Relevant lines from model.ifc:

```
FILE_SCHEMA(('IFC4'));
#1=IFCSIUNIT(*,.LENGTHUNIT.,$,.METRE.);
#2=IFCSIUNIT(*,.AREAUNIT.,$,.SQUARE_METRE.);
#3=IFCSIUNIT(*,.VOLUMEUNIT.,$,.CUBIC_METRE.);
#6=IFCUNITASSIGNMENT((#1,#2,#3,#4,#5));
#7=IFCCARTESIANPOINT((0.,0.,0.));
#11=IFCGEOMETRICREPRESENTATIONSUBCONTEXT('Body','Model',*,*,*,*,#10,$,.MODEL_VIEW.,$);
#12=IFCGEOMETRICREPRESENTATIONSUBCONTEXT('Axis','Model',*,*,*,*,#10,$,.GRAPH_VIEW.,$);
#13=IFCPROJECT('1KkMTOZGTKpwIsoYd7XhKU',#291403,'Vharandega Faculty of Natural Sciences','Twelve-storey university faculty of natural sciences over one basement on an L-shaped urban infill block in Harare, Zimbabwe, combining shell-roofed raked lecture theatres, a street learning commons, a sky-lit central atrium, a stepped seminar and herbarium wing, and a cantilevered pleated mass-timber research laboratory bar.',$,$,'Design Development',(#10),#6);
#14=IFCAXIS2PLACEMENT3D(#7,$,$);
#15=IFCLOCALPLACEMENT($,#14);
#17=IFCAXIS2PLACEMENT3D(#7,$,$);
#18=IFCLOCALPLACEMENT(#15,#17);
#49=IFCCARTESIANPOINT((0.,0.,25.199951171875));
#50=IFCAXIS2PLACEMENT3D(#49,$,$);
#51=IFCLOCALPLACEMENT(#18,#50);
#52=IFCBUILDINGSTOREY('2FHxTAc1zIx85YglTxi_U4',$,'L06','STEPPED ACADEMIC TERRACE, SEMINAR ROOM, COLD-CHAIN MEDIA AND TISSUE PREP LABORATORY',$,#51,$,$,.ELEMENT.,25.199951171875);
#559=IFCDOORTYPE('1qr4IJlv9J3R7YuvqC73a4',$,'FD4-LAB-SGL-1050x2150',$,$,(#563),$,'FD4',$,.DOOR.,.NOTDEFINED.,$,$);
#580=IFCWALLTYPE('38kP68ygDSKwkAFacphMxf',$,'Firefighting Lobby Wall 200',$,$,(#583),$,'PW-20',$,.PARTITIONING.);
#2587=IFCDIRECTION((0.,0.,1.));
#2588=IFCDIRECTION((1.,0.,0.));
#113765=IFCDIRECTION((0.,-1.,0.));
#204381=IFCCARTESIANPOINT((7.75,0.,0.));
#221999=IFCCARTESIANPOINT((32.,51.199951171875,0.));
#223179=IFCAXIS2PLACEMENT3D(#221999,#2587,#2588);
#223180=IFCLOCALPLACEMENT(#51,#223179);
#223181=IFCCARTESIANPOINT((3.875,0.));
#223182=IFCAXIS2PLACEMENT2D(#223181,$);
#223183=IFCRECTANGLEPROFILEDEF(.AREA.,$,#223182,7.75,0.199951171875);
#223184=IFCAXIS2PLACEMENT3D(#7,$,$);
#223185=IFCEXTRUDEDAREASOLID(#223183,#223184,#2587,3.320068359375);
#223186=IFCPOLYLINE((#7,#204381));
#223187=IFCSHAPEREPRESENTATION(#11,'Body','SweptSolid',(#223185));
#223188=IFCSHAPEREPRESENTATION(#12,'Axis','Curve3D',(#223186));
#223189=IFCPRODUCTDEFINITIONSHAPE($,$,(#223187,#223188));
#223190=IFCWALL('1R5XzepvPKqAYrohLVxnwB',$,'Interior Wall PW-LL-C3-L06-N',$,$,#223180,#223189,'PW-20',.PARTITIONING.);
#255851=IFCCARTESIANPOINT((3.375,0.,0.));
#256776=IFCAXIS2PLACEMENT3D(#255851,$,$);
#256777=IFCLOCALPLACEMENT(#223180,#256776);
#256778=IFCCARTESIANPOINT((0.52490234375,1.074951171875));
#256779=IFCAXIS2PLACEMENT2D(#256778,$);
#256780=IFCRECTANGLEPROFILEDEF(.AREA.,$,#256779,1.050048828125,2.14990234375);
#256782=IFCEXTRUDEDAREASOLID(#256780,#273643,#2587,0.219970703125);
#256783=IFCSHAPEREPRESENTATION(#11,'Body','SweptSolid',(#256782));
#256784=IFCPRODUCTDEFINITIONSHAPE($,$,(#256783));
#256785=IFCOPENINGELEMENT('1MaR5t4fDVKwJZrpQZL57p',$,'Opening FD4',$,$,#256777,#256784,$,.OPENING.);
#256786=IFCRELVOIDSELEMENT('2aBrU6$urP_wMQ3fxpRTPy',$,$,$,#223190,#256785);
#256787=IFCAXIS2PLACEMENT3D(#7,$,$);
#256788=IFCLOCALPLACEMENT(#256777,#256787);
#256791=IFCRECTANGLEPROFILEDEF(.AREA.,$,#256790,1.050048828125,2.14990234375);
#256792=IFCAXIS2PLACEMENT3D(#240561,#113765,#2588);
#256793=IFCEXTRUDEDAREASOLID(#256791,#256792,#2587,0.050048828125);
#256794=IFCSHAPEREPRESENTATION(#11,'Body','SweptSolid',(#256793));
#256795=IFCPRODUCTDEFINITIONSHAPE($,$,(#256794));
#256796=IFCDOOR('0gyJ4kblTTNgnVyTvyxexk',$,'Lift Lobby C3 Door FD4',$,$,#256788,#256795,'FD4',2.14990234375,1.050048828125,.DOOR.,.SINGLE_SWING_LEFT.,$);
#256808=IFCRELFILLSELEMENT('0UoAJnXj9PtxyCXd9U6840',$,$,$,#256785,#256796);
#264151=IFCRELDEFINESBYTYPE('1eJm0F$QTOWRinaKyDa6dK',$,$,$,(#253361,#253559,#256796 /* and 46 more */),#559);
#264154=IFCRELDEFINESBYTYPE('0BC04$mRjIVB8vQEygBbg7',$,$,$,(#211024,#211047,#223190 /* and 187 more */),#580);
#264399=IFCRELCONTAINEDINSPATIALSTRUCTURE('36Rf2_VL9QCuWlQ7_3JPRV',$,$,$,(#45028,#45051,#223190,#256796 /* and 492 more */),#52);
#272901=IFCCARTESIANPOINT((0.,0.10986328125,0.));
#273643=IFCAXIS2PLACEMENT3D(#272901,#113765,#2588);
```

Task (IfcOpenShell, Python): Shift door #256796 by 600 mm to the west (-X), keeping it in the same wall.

```python
import ifcopenshell
import ifcopenshell.api.geometry
import ifcopenshell.util.placement

model = ifcopenshell.open("model.ifc")

door = model.by_guid("0gyJ4kblTTNgnVyTvyxexk")
opening = door.FillsVoids[0].RelatingOpeningElement
wall = opening.VoidsElements[0].RelatingBuildingElement

wall_matrix = ifcopenshell.util.placement.get_local_placement(wall.ObjectPlacement)
shift = wall_matrix[:3, 0] * -0.6
before = ifcopenshell.util.placement.get_local_placement(door.ObjectPlacement)[:3, 3].copy()

# The door is placed relative to its opening, so it follows when the opening moves.
matrix = ifcopenshell.util.placement.get_local_placement(opening.ObjectPlacement)
matrix[:3, 3] += shift
ifcopenshell.api.geometry.edit_object_placement(
    model, product=opening, matrix=matrix, is_si=False, should_transform_children=True
)

after = ifcopenshell.util.placement.get_local_placement(door.ObjectPlacement)[:3, 3]
print("door moved by", (after - before).round(3) + 0.0)

model.write("model_updated.ifc")
```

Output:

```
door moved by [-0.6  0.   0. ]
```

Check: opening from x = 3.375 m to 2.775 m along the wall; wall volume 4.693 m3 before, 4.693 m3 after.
